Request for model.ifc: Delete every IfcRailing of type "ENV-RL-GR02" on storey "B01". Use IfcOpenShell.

First a look at what the model holds.

```python
import ifcopenshell
import ifcopenshell.util.element

model = ifcopenshell.open("model.ifc")
print(model.schema)
storey = next(s for s in model.by_type("IfcBuildingStorey") if s.Name == "B01")
railings = [e for e in ifcopenshell.util.element.get_decomposition(storey) if e.is_a("IfcRailing")]
seen = {}
for e in railings:
    element_type = ifcopenshell.util.element.get_type(e)
    name = element_type.Name if element_type not in (None, e) else None
    seen[name] = seen.get(name, 0) + 1
for name, count in sorted(seen.items(), key=str):
    print(count, "x", name)
```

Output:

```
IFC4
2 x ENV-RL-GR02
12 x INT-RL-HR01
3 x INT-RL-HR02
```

```python
import ifcopenshell
import ifcopenshell.api.root
import ifcopenshell.util.element

model = ifcopenshell.open("model.ifc")

storey = next(s for s in model.by_type("IfcBuildingStorey") if s.Name == "B01")
railings = [e for e in ifcopenshell.util.element.get_decomposition(storey) if e.is_a("IfcRailing")]
targets = [e for e in railings if (t := ifcopenshell.util.element.get_type(e)) not in (None, e) and t.Name == "ENV-RL-GR02"]

for e in targets:
    ifcopenshell.api.root.remove_product(model, product=e)
print(len(targets), "removed")

model.write("model_updated.ifc")
```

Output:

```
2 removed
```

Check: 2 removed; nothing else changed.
